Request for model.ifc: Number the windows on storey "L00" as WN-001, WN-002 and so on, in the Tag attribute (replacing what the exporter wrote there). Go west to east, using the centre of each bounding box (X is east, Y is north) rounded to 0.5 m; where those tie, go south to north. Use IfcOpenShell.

First a look at what the model holds.

```python
import ifcopenshell
import ifcopenshell.util.element
import ifcopenshell.util.placement

model = ifcopenshell.open("model.ifc")
print(model.schema)
storey = next(s for s in model.by_type("IfcBuildingStorey") if s.Name == "L00")
windows = [e for e in ifcopenshell.util.element.get_decomposition(storey) if e.is_a("IfcWindow")]
for e in sorted(windows, key=lambda e: e.id()):
    origin = ifcopenshell.util.placement.get_local_placement(e.ObjectPlacement)[:3, 3]
    print(e.id(), e.Tag, e.Name, origin.round(2) + 0.0, sep=" | ")
```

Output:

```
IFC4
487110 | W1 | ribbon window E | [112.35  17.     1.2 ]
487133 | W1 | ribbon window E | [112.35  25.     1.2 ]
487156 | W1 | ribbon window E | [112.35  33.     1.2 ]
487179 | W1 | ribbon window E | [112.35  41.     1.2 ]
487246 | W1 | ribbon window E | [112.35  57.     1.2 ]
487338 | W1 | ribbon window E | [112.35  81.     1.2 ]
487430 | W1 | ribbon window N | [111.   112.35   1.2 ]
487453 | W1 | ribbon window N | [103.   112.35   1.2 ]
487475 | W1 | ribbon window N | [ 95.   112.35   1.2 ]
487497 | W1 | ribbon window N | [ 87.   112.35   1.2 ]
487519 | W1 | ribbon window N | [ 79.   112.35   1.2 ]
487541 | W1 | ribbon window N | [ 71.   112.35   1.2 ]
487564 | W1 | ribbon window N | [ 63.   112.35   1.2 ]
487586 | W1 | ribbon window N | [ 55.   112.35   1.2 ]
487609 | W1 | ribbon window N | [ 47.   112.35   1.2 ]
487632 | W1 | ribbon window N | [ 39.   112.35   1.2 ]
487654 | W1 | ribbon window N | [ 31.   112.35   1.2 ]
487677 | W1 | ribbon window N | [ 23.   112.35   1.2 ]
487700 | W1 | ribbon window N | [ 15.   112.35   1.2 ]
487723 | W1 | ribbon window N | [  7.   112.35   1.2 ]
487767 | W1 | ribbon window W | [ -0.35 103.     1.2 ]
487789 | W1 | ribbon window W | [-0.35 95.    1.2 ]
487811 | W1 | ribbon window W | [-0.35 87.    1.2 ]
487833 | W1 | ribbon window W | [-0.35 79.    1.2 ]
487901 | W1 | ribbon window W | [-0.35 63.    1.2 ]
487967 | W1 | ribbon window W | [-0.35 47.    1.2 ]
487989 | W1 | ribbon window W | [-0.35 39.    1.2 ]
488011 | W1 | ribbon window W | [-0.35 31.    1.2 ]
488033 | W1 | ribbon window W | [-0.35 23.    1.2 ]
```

```python
import ifcopenshell
import ifcopenshell.geom
import ifcopenshell.util.element
import ifcopenshell.util.shape

model = ifcopenshell.open("model.ifc")
settings = ifcopenshell.geom.settings()
settings.set("use-world-coords", True)


def centre(element):
    shape = ifcopenshell.geom.create_shape(settings, element)
    return ifcopenshell.util.shape.get_bbox_centroid(shape.geometry)


storey = next(s for s in model.by_type("IfcBuildingStorey") if s.Name == "L00")
windows = [e for e in ifcopenshell.util.element.get_decomposition(storey) if e.is_a("IfcWindow")]

# Insertion points can sit at a corner or the storey origin, so sort by the geometry (in metres).
centres = {e: centre(e) for e in windows}
windows.sort(key=lambda e: (round(centres[e][0] / 0.5), centres[e][1]))

for i, e in enumerate(windows, start=1):
    number = f"WN-0{i:02d}"
    e.Tag = number
    print(e.id(), number)

model.write("model_rev.ifc")
```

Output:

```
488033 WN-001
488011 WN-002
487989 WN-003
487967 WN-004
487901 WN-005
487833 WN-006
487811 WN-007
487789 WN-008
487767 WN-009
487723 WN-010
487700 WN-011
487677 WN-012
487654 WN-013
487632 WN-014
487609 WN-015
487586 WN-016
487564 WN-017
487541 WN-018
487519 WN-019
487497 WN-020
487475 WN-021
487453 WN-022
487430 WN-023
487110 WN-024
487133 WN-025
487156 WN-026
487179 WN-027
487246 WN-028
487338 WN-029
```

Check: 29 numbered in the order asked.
